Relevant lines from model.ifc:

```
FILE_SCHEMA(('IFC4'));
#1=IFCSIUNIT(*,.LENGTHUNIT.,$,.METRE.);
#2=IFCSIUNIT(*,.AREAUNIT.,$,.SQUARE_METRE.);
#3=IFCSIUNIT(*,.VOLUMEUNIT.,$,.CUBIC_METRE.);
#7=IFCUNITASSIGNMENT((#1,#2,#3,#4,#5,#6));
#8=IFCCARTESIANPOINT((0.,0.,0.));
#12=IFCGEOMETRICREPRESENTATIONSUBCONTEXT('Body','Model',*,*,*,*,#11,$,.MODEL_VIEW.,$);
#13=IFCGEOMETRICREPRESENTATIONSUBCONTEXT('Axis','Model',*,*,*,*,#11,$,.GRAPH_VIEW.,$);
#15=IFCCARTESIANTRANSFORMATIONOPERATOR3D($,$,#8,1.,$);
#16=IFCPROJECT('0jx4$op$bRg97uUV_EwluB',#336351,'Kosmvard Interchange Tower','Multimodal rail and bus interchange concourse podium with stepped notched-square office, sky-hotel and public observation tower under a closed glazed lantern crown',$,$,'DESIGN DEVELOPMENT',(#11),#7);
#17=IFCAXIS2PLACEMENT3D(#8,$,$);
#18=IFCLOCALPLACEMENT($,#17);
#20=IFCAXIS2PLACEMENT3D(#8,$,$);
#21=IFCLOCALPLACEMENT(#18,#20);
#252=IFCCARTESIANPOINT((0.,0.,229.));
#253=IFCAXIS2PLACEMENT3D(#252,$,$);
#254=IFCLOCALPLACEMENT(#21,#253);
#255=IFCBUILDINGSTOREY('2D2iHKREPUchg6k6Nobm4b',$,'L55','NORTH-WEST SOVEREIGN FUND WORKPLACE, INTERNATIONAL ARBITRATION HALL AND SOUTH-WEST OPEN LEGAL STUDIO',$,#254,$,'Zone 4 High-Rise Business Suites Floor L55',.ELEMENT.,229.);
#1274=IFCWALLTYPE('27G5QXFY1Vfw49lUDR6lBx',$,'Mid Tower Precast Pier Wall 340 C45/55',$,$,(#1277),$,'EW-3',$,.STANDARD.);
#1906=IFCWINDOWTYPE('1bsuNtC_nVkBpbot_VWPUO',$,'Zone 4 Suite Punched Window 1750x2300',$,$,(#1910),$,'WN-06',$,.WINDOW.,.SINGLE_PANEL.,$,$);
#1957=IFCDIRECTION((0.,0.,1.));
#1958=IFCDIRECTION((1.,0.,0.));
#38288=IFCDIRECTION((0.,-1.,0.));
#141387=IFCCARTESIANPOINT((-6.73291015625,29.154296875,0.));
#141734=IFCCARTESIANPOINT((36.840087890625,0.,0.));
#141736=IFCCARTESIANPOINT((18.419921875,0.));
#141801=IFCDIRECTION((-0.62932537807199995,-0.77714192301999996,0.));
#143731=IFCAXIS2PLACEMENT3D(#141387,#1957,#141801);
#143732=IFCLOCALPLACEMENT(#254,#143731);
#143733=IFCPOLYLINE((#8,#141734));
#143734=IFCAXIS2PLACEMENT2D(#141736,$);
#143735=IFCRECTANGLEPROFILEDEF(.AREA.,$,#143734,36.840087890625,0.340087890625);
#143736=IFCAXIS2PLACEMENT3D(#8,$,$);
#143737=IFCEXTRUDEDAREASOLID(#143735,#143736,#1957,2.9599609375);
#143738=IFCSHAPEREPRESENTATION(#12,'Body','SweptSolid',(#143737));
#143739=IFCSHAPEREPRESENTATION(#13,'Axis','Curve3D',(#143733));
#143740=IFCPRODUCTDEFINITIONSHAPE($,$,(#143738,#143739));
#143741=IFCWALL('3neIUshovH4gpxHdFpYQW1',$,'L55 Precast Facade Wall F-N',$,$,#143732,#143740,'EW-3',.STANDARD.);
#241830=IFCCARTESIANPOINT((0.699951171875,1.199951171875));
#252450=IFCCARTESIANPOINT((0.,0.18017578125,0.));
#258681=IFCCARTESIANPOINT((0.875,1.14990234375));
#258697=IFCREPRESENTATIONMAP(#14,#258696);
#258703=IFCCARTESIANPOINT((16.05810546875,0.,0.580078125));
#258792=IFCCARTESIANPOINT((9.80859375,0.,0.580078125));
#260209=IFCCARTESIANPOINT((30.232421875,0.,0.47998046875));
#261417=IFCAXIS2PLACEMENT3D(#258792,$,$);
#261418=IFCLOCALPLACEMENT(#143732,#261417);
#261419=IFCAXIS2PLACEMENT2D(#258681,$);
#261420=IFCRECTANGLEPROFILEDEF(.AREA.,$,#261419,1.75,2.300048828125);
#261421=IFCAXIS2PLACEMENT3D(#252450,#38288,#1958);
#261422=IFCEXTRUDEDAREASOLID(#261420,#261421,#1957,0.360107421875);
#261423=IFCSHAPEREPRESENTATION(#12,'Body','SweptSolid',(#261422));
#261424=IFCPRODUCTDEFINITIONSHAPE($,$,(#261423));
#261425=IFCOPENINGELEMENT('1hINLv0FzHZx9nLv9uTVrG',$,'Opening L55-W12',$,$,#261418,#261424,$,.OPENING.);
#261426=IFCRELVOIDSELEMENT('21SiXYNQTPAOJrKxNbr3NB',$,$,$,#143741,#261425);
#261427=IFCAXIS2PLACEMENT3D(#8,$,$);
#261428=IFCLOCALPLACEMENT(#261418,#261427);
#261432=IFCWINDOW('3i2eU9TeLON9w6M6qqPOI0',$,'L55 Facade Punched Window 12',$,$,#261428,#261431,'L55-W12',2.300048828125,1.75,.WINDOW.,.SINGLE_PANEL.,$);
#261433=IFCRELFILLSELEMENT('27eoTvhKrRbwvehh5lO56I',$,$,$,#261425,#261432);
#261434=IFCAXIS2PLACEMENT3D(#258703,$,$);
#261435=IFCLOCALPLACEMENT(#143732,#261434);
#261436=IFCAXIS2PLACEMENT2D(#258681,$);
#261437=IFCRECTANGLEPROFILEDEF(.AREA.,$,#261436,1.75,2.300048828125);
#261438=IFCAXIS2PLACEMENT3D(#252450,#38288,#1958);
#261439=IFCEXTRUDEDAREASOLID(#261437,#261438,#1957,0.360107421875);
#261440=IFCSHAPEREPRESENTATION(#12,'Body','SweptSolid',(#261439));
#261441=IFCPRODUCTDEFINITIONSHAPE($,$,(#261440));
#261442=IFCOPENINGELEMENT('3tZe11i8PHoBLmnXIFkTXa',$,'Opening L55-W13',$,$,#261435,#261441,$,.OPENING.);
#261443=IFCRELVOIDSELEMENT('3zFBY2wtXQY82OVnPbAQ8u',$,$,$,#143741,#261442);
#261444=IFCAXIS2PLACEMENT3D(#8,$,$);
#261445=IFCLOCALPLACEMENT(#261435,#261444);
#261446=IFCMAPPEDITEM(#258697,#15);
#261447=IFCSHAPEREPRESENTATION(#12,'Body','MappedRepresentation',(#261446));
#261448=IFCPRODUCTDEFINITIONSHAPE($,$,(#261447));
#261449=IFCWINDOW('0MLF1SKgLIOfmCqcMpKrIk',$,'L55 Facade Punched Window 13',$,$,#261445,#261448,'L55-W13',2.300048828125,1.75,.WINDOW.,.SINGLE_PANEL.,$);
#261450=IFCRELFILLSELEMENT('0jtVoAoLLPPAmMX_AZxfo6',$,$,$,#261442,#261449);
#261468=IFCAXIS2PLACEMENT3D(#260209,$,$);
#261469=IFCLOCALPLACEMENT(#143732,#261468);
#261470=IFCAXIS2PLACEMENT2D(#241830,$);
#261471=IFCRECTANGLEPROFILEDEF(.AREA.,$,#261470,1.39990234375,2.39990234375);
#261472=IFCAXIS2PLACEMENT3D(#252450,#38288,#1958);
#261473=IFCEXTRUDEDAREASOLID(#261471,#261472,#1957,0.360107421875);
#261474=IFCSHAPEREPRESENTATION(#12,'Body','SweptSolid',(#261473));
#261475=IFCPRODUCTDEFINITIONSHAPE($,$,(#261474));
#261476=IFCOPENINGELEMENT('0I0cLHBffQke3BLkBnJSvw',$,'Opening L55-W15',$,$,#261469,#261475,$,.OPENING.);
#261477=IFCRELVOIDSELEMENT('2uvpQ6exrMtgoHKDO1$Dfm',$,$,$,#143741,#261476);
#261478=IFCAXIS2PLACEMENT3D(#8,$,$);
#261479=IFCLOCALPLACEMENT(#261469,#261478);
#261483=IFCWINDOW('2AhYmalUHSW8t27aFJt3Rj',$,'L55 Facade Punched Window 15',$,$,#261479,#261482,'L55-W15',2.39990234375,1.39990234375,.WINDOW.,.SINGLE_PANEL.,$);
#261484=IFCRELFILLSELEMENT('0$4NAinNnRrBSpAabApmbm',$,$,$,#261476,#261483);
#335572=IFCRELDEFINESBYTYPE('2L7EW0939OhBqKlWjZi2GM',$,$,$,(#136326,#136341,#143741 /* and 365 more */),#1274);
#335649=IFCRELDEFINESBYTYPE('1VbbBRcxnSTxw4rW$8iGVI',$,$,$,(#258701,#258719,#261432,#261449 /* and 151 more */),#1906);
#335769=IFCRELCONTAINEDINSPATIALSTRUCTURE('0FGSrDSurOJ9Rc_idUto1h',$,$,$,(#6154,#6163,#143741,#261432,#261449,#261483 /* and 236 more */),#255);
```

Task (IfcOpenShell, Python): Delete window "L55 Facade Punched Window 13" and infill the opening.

```python
import ifcopenshell
import ifcopenshell.api.feature
import ifcopenshell.api.root
import ifcopenshell.geom
import ifcopenshell.util.shape

model = ifcopenshell.open("model.ifc")
settings = ifcopenshell.geom.settings()


def volume(element):
    """Net volume in cubic metres, openings subtracted."""
    shape = ifcopenshell.geom.create_shape(settings, element)
    return ifcopenshell.util.shape.get_volume(shape.geometry)


window = model.by_id(261449)
opening = window.FillsVoids[0].RelatingOpeningElement
wall = opening.VoidsElements[0].RelatingBuildingElement
before = volume(wall)

ifcopenshell.api.root.remove_product(model, product=window)
ifcopenshell.api.feature.remove_feature(model, feature=opening)

after = volume(wall)

print(f"wall volume {before:.3f} -> {after:.3f} m3")

model.write("model_v2.ifc")
```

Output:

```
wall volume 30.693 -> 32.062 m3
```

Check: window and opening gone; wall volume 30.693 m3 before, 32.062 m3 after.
